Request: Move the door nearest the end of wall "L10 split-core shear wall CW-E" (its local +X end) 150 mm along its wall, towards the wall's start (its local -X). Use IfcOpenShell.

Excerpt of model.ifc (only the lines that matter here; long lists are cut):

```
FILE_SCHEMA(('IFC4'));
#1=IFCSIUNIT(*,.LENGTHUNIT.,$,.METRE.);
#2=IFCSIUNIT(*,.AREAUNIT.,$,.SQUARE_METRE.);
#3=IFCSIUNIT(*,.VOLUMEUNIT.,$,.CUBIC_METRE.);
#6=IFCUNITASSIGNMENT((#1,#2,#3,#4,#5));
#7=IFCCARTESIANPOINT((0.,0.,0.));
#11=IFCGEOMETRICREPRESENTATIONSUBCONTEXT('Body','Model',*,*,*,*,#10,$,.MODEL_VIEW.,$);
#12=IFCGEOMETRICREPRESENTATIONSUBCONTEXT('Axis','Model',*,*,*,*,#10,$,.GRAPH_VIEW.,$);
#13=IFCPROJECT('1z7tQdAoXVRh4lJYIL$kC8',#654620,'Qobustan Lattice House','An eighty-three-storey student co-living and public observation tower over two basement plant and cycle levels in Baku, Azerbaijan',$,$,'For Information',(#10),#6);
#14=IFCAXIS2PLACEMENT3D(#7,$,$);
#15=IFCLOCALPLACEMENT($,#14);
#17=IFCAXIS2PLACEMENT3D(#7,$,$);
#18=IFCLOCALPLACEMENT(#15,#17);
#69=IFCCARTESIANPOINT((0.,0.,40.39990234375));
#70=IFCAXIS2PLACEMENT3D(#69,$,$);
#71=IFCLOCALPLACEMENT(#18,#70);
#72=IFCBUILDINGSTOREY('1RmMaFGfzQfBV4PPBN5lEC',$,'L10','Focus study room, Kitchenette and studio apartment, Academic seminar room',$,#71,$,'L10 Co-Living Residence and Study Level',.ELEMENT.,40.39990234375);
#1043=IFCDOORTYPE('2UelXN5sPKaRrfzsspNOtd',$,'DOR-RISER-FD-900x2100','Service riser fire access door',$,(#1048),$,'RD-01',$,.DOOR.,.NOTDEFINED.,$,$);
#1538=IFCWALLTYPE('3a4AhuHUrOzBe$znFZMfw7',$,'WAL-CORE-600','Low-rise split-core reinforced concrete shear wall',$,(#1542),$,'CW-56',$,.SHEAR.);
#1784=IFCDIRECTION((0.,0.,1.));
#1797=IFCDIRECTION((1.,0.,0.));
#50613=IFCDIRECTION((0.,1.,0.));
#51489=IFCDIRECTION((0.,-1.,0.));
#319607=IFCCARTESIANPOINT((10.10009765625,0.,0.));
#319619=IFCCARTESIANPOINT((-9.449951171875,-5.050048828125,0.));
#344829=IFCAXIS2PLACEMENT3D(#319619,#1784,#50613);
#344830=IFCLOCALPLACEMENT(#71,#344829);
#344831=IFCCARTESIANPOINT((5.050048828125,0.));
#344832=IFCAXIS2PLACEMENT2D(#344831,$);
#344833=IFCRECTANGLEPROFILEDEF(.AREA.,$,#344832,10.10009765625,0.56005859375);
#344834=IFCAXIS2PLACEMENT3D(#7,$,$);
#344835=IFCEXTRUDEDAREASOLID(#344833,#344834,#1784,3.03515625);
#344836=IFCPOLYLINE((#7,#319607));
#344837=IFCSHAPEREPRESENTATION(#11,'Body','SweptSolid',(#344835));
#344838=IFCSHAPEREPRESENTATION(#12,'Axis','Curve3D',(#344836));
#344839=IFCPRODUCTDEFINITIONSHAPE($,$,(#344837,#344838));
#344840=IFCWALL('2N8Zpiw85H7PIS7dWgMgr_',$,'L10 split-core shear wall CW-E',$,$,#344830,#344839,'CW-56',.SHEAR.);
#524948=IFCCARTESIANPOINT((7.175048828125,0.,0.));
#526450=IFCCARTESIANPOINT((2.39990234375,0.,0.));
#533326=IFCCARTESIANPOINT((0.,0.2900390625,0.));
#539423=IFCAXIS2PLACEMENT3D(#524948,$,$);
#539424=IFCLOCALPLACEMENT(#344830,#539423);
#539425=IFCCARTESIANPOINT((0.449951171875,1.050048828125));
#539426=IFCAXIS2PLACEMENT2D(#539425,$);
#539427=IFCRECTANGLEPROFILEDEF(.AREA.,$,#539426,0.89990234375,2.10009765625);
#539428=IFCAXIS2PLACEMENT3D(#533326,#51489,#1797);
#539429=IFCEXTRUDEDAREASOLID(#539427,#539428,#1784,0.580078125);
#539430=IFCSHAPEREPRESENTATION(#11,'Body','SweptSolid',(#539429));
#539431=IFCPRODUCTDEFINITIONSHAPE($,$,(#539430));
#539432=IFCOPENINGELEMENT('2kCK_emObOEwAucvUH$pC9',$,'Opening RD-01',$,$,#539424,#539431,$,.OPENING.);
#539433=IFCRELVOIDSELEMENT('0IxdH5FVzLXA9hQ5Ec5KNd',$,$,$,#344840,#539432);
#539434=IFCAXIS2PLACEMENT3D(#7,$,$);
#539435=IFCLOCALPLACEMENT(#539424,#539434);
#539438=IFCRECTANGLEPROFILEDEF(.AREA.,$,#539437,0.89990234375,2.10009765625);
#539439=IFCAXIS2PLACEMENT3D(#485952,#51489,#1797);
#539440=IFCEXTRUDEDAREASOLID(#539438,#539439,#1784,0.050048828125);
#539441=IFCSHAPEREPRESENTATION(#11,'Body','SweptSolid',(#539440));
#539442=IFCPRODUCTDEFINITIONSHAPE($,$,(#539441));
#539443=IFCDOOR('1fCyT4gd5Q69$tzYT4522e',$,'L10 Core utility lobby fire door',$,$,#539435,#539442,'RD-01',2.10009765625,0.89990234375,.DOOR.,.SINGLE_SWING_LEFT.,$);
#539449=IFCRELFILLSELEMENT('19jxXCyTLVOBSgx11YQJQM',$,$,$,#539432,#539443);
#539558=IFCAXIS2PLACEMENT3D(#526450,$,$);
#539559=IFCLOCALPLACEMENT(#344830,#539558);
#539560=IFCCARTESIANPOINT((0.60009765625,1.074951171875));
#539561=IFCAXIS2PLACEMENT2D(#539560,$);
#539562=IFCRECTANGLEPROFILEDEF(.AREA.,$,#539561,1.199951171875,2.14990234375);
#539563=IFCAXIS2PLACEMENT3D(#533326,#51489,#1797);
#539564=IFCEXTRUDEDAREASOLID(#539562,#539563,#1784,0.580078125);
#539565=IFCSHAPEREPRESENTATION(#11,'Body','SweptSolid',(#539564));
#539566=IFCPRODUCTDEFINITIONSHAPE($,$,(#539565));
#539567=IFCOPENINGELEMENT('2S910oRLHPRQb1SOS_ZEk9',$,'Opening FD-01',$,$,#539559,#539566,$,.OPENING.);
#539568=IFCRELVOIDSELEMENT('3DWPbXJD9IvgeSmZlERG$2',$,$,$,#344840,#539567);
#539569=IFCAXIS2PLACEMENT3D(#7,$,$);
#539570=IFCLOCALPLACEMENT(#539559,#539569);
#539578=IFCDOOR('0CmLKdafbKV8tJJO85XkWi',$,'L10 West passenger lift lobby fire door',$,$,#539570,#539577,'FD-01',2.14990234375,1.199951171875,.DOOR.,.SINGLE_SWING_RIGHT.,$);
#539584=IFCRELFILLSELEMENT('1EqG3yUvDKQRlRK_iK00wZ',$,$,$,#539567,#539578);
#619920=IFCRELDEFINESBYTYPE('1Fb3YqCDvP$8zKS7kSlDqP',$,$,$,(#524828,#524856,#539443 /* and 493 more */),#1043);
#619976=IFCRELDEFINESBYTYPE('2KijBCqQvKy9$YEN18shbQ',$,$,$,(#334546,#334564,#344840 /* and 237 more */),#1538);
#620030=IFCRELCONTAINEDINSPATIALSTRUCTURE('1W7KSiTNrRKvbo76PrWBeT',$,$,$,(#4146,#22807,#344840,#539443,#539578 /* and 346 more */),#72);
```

```python
import ifcopenshell
import ifcopenshell.api.geometry
import ifcopenshell.util.placement
import ifcopenshell.util.unit

model = ifcopenshell.open("model.ifc")
unit_scale = ifcopenshell.util.unit.calculate_unit_scale(model)

door = model.by_guid("1fCyT4gd5Q69$tzYT4522e")
opening = door.FillsVoids[0].RelatingOpeningElement
wall = opening.VoidsElements[0].RelatingBuildingElement

wall_matrix = ifcopenshell.util.placement.get_local_placement(wall.ObjectPlacement)
shift = wall_matrix[:3, 0] * -0.15 / unit_scale
before = ifcopenshell.util.placement.get_local_placement(door.ObjectPlacement)[:3, 3].copy()

# The door is placed relative to its opening, so it follows when the opening moves.
matrix = ifcopenshell.util.placement.get_local_placement(opening.ObjectPlacement)
matrix[:3, 3] += shift
ifcopenshell.api.geometry.edit_object_placement(
    model, product=opening, matrix=matrix, is_si=False, should_transform_children=True
)

after = ifcopenshell.util.placement.get_local_placement(door.ObjectPlacement)[:3, 3]
print("door moved by", (after - before).round(3) + 0.0)

model.write("model_updated.ifc")
```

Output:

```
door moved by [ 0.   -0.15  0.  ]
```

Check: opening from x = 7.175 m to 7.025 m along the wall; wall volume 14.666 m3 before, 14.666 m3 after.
